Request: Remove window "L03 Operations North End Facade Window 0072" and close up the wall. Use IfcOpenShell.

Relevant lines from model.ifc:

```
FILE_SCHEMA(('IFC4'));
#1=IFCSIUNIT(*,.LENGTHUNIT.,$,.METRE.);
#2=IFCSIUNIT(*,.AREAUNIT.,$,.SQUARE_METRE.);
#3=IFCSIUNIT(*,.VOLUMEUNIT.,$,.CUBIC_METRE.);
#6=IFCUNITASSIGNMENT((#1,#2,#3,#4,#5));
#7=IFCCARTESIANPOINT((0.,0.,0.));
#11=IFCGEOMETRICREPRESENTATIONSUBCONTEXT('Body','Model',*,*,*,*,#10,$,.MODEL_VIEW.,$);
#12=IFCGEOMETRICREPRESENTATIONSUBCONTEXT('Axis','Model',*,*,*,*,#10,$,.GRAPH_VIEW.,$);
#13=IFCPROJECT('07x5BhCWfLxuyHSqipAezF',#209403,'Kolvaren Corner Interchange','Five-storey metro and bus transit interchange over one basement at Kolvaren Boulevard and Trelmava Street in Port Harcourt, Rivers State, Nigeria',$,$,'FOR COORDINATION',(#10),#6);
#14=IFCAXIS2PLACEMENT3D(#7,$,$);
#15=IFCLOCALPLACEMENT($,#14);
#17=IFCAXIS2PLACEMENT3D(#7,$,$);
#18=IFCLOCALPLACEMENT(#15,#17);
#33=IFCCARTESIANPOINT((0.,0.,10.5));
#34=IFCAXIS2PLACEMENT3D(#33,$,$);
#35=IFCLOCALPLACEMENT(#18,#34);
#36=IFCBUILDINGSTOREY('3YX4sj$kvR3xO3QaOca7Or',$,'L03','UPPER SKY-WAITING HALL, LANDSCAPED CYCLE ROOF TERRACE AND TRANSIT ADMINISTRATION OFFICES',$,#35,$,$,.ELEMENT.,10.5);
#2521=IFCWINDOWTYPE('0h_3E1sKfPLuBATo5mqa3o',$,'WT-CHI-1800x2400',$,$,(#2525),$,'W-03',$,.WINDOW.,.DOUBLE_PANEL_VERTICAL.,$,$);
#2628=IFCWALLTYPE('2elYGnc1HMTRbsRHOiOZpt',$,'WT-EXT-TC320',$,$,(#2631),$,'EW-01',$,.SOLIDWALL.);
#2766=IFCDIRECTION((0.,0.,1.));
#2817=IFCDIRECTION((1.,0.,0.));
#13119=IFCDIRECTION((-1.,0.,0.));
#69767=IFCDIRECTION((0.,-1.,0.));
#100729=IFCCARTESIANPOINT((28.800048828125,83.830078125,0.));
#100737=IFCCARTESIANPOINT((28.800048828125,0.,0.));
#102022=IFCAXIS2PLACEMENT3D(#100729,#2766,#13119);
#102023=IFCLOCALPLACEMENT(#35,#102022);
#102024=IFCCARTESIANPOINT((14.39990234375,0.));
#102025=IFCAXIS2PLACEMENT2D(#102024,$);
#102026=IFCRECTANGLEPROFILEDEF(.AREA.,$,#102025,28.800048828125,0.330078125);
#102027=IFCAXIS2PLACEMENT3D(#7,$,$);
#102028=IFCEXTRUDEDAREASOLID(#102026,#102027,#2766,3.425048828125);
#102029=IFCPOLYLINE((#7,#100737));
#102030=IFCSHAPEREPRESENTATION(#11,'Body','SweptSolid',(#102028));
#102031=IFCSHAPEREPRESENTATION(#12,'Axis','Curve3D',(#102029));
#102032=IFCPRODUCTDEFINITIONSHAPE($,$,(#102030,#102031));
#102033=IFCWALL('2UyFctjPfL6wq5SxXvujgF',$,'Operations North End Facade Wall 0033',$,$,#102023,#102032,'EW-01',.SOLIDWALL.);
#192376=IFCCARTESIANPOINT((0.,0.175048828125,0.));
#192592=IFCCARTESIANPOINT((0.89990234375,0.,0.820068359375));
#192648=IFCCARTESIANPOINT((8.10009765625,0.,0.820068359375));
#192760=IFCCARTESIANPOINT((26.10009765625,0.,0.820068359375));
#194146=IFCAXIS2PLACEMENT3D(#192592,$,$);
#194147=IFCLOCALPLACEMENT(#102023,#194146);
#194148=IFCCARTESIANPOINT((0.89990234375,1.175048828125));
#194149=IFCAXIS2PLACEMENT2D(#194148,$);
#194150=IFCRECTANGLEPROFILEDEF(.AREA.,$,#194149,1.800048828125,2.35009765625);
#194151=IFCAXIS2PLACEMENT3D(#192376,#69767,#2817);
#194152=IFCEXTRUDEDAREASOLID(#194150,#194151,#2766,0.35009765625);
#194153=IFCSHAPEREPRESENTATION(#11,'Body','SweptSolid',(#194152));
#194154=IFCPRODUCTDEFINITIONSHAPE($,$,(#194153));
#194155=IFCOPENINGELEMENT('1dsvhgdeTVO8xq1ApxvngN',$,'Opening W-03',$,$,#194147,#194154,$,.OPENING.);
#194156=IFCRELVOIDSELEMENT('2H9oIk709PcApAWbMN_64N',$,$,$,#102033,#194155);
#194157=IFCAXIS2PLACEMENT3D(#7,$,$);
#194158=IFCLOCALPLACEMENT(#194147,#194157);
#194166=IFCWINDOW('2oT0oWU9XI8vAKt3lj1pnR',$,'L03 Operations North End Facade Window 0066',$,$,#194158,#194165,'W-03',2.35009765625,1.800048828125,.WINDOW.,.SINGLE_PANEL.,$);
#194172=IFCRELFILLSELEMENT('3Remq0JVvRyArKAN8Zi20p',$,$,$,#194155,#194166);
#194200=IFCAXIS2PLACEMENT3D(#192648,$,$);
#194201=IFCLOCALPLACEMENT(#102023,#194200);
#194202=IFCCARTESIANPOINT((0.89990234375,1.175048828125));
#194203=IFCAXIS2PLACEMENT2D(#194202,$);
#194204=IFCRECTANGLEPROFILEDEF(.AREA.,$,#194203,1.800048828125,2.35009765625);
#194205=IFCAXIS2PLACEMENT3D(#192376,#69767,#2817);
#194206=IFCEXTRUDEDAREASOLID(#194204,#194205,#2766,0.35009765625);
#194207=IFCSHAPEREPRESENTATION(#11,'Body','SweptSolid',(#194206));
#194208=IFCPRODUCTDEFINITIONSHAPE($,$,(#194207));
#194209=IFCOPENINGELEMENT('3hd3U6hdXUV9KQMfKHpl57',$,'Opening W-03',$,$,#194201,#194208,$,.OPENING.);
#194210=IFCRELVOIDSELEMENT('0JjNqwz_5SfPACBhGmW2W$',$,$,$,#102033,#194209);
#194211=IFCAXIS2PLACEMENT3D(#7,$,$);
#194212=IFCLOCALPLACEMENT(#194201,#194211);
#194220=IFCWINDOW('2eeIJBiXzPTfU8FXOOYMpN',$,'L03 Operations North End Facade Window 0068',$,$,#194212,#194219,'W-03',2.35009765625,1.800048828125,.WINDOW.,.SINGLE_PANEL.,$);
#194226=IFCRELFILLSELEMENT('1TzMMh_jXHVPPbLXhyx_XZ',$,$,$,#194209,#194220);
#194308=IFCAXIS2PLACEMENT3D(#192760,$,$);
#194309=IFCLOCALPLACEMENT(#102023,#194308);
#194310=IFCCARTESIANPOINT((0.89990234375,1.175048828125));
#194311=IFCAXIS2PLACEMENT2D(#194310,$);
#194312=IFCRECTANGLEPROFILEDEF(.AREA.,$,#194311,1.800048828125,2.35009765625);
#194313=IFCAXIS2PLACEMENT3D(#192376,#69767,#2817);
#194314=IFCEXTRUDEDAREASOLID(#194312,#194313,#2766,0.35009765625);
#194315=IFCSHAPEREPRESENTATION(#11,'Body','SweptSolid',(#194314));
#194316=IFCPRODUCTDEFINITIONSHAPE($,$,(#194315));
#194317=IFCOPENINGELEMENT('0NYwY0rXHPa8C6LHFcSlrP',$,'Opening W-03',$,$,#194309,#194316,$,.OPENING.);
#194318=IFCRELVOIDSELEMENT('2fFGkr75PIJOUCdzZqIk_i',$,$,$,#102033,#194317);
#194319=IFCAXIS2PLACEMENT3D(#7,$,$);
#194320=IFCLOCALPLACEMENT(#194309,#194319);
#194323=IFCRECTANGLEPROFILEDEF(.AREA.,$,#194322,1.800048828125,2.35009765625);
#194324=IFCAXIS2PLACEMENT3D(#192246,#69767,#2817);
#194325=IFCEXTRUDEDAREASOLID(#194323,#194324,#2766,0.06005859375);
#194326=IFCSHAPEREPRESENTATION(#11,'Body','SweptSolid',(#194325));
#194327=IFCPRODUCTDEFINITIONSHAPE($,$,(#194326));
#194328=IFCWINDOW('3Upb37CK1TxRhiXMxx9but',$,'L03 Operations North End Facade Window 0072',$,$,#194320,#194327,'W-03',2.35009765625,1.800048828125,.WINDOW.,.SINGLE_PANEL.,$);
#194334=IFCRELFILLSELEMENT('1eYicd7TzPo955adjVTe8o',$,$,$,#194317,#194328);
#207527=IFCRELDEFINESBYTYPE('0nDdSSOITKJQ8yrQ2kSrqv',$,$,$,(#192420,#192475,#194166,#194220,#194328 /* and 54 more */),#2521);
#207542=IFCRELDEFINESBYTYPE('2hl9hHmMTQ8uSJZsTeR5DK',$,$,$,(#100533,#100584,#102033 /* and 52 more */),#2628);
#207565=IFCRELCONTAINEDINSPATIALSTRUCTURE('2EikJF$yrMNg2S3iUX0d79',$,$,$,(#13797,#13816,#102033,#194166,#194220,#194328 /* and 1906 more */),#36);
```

```python
import ifcopenshell
import ifcopenshell.api.feature
import ifcopenshell.api.root
import ifcopenshell.geom
import ifcopenshell.util.shape

model = ifcopenshell.open("model.ifc")
settings = ifcopenshell.geom.settings()


def volume(element):
    """Net volume in cubic metres, openings subtracted."""
    shape = ifcopenshell.geom.create_shape(settings, element)
    return ifcopenshell.util.shape.get_volume(shape.geometry)


window = model.by_id(194328)
opening = window.FillsVoids[0].RelatingOpeningElement
wall = opening.VoidsElements[0].RelatingBuildingElement
before = volume(wall)

ifcopenshell.api.root.remove_product(model, product=window)
ifcopenshell.api.feature.remove_feature(model, feature=opening)

after = volume(wall)

print(f"wall volume {before:.3f} -> {after:.3f} m3")

model.write("model_updated.ifc")
```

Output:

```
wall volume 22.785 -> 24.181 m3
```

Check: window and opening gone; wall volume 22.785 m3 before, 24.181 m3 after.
